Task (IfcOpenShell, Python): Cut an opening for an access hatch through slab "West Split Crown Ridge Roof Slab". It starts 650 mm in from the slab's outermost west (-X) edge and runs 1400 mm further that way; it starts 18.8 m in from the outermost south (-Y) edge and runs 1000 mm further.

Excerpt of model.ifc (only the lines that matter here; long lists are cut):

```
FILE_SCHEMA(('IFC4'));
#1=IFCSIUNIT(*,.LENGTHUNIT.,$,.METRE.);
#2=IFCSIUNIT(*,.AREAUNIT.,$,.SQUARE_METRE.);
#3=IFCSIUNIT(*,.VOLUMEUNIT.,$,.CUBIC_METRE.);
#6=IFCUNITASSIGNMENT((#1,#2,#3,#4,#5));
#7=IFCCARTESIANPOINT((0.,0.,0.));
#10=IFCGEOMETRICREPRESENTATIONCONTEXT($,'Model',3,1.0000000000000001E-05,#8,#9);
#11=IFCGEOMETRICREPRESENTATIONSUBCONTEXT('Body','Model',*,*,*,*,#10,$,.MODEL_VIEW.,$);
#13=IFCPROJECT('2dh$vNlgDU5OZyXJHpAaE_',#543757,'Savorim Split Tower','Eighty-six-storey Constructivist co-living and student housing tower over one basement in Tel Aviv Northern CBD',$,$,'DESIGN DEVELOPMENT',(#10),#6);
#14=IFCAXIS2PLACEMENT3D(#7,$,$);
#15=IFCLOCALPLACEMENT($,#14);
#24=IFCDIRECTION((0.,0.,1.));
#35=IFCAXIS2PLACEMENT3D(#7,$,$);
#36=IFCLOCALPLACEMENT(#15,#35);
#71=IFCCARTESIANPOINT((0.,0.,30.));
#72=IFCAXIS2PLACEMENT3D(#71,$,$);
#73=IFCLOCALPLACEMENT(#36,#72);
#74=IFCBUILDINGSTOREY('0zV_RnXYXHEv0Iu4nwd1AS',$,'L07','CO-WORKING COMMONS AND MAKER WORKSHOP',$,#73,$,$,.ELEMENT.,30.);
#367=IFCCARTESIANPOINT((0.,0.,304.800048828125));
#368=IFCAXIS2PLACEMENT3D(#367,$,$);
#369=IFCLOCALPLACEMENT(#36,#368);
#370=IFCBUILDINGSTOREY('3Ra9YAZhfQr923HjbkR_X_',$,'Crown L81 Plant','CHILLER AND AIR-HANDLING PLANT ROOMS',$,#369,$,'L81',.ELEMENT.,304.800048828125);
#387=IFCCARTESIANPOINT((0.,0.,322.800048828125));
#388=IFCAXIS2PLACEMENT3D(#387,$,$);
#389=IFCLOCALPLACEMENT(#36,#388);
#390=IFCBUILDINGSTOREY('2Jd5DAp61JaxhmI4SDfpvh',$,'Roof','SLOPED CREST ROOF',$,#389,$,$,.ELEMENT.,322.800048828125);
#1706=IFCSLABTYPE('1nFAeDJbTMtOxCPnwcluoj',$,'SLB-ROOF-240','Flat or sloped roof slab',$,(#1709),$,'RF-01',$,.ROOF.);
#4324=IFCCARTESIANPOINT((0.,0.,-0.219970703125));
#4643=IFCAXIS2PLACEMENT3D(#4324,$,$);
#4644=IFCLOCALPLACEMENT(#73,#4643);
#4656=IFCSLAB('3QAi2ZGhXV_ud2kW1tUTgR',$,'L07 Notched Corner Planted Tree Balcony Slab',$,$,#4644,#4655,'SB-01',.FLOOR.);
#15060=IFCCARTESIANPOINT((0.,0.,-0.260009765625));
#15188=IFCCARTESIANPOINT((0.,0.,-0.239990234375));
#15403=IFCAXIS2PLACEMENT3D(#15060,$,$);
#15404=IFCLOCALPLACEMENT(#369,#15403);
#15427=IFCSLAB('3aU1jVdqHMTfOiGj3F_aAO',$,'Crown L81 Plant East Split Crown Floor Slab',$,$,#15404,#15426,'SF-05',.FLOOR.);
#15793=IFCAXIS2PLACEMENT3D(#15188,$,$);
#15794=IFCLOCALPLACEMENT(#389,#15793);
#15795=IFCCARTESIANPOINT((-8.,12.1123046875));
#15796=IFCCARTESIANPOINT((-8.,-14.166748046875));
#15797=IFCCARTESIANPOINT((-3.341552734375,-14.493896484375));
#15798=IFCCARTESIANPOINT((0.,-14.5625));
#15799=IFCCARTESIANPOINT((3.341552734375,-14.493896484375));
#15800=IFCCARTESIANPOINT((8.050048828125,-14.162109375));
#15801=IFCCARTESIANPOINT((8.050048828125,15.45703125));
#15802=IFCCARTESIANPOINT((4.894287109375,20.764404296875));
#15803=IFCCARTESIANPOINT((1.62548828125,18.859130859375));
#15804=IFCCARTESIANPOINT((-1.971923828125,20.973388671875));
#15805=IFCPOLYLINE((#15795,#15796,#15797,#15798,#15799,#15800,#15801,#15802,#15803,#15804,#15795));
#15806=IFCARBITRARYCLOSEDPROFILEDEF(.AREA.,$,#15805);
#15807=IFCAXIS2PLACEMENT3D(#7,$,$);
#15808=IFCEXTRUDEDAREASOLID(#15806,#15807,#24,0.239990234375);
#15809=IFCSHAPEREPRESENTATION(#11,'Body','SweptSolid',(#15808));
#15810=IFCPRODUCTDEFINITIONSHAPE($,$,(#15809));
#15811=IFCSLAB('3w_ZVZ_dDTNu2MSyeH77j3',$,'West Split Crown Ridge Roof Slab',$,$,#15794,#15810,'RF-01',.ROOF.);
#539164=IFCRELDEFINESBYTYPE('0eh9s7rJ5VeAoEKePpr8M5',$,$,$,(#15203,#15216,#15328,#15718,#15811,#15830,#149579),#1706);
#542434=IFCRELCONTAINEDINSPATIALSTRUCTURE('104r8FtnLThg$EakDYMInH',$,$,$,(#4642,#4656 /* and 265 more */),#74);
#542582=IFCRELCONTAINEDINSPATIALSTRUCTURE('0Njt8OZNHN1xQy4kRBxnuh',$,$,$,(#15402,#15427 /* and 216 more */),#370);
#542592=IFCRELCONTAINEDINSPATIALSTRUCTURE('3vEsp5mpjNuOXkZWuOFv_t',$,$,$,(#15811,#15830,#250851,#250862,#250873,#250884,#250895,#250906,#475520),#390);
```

```python
import numpy as np
import ifcopenshell
import ifcopenshell.api.feature
import ifcopenshell.api.geometry
import ifcopenshell.api.root
import ifcopenshell.geom
import ifcopenshell.util.placement
import ifcopenshell.util.representation
import ifcopenshell.util.shape
import ifcopenshell.util.unit

model = ifcopenshell.open("model.ifc")
unit_scale = ifcopenshell.util.unit.calculate_unit_scale(model)
settings = ifcopenshell.geom.settings()


def volume(element):
    """Net volume in cubic metres, openings subtracted."""
    shape = ifcopenshell.geom.create_shape(settings, element)
    return ifcopenshell.util.shape.get_volume(shape.geometry)


slab = model.by_guid("3w_ZVZ_dDTNu2MSyeH77j3")
before = volume(slab)

# Extent in the slab's own axes, in metres. The edges named are its -X and -Y sides.
slab_shape = ifcopenshell.geom.create_shape(settings, slab)
vertices = ifcopenshell.util.shape.get_vertices(slab_shape.geometry)
x_min, y_min, bottom = vertices.min(axis=0)
top = vertices[:, 2].max()

opening = ifcopenshell.api.root.create_entity(model, ifc_class="IfcOpeningElement", name="Access hatch opening", predefined_type="OPENING")
context = ifcopenshell.util.representation.get_context(model, "Model", "Body", "MODEL_VIEW")
width, depth = 1.4, 1
outline = [(0.0, 0.0), (width, 0.0), (width, depth), (0.0, depth), (0.0, 0.0)]
# Overshoot both faces by 50 mm so the cut is clean.
shape = ifcopenshell.api.geometry.add_slab_representation(
    model, context=context, depth=top - bottom + 0.1, polyline=outline
)
ifcopenshell.api.geometry.assign_representation(model, product=opening, representation=shape)

matrix = ifcopenshell.util.placement.get_local_placement(slab.ObjectPlacement)
matrix[:, 3] = matrix @ np.append(np.array([x_min + 0.65, y_min + 18.8, bottom - 0.05]) / unit_scale, 1.0)
ifcopenshell.api.geometry.edit_object_placement(model, product=opening, matrix=matrix, is_si=False)
ifcopenshell.api.feature.add_feature(model, feature=opening, element=slab)

after = volume(slab)

print(f"slab volume {before:.3f} -> {after:.3f} m3")

model.write("model_updated.ifc")
```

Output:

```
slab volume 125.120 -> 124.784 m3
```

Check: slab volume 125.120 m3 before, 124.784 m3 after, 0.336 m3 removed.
